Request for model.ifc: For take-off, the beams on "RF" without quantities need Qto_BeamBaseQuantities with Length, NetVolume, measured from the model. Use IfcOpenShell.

First a look at what the model holds.

```python
import ifcopenshell
import ifcopenshell.util.element
import ifcopenshell.util.unit

model = ifcopenshell.open("model.ifc")
print(model.schema)
for unit_type in ("LENGTHUNIT", "AREAUNIT", "VOLUMEUNIT"):
    print(unit_type, ifcopenshell.util.unit.calculate_unit_scale(model, unit_type))
storey = next(s for s in model.by_type("IfcBuildingStorey") if s.Name == "RF")
beams = [e for e in ifcopenshell.util.element.get_decomposition(storey) if e.is_a("IfcBeam")]
for e in sorted(beams, key=lambda e: e.id()):
    print(e.id(), e.is_a(), e.Name, list(ifcopenshell.util.element.get_psets(e, qtos_only=True)), sep=" | ")
```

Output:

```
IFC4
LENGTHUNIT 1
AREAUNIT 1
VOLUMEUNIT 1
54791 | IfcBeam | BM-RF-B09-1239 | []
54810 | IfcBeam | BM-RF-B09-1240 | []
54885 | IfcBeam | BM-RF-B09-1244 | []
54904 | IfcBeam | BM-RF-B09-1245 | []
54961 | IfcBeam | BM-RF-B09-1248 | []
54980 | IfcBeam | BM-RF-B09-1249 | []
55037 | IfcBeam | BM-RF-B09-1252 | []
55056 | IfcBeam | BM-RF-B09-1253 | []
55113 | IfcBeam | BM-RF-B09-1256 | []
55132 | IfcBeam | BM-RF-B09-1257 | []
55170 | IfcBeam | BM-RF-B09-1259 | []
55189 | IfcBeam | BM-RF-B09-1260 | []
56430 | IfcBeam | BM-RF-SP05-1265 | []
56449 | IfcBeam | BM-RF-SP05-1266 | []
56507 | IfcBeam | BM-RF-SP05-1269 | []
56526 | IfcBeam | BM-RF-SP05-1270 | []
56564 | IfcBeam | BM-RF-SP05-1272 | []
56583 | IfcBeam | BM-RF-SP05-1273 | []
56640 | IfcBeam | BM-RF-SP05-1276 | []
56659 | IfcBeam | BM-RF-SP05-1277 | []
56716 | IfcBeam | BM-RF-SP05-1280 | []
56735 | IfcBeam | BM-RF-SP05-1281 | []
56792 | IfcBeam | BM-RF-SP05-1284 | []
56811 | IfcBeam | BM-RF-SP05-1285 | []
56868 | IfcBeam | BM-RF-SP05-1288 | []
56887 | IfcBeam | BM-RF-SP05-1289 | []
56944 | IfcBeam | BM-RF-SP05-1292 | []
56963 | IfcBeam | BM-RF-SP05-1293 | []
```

```python
import ifcopenshell
import ifcopenshell.api.pset
import ifcopenshell.geom
import ifcopenshell.util.element
import ifcopenshell.util.shape
import ifcopenshell.util.unit

model = ifcopenshell.open("model.ifc")
unit_scale = ifcopenshell.util.unit.calculate_unit_scale(model)
volume_scale = ifcopenshell.util.unit.calculate_unit_scale(model, "VOLUMEUNIT")
settings = ifcopenshell.geom.settings()

storey = next(s for s in model.by_type("IfcBuildingStorey") if s.Name == "RF")
beams = [e for e in ifcopenshell.util.element.get_decomposition(storey) if e.is_a("IfcBeam")]

for e in sorted(beams, key=lambda e: e.id()):
    if ifcopenshell.util.element.get_psets(e, qtos_only=True, should_inherit=False):
        continue
    # Geometry comes back in metres, in the element's own axes.
    shape = ifcopenshell.geom.create_shape(settings, e)
    values = {
        "Length": ifcopenshell.util.shape.get_max_xyz(shape.geometry) / unit_scale,
        "NetVolume": ifcopenshell.util.shape.get_volume(shape.geometry) / volume_scale,
    }
    qto = ifcopenshell.api.pset.add_qto(model, product=e, name="Qto_BeamBaseQuantities")
    ifcopenshell.api.pset.edit_qto(model, qto=qto, properties=values)
    print(e.id(), {k: round(v, 3) for k, v in values.items()})

model.write("model-out.ifc")
```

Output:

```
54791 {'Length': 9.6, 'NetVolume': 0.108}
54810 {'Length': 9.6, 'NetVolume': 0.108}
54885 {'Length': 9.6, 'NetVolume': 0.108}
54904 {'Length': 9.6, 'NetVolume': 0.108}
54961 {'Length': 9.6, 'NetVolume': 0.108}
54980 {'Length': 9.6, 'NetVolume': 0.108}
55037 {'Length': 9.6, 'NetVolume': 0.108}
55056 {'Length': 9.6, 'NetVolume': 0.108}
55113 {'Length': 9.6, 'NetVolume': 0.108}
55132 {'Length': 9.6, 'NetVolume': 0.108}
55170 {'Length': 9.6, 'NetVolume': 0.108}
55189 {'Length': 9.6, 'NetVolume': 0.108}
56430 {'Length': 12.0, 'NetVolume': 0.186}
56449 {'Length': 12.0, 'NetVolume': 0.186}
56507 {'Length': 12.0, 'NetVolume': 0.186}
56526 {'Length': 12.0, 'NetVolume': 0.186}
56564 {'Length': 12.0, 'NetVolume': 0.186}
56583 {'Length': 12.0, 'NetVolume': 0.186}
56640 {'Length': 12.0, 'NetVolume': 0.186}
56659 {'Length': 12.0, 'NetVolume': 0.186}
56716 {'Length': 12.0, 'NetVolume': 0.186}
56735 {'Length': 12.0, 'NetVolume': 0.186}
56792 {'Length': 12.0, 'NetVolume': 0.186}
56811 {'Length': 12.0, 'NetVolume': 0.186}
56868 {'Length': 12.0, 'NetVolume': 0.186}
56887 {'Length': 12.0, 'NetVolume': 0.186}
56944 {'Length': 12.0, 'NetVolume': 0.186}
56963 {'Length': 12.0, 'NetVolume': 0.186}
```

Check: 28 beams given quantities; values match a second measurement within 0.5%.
